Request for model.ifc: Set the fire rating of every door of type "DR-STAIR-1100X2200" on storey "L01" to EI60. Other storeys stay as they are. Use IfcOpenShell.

First a look at what the model holds.

```python
import ifcopenshell
import ifcopenshell.util.element

model = ifcopenshell.open("model.ifc")
print(model.schema)
storey = next(s for s in model.by_type("IfcBuildingStorey") if s.Name == "L01")
doors = [e for e in ifcopenshell.util.element.get_decomposition(storey) if e.is_a("IfcDoor")]
seen = {}
for e in doors:
    element_type = ifcopenshell.util.element.get_type(e)
    key = (element_type.Name if element_type != e and element_type else None, ifcopenshell.util.element.get_pset(e, "Pset_DoorCommon", "FireRating"))
    seen[key] = seen.get(key, 0) + 1
for (name, value), count in sorted(seen.items(), key=str):
    print(count, "x", name, "|", value)
```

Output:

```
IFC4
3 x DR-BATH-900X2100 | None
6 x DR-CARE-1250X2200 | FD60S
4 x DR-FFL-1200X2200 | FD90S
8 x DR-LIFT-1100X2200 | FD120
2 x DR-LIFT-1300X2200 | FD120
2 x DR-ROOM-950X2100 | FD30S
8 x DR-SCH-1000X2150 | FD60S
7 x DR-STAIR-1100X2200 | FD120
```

```python
import ifcopenshell
import ifcopenshell.api.pset
import ifcopenshell.util.element

model = ifcopenshell.open("model.ifc")

storey = next(s for s in model.by_type("IfcBuildingStorey") if s.Name == "L01")
doors = [e for e in ifcopenshell.util.element.get_decomposition(storey) if e.is_a("IfcDoor")]

count = 0
for e in doors:
    element_type = ifcopenshell.util.element.get_type(e)
    if element_type in (None, e) or element_type.Name != "DR-STAIR-1100X2200":
        continue
    found = ifcopenshell.util.element.get_pset(e, "Pset_DoorCommon", should_inherit=False)
    if found:
        pset = model.by_id(found["id"])
        if len(ifcopenshell.util.element.get_elements_by_pset(pset)) > 1:
            pset = ifcopenshell.api.pset.unshare_pset(model, products=[e], pset=pset)[0]
    else:
        pset = ifcopenshell.api.pset.add_pset(model, product=e, name="Pset_DoorCommon")
    ifcopenshell.api.pset.edit_pset(model, pset=pset, properties={"FireRating": "EI60"})
    count += 1

print(count, "doors updated")

model.write("model_rev.ifc")
```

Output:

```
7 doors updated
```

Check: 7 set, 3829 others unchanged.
